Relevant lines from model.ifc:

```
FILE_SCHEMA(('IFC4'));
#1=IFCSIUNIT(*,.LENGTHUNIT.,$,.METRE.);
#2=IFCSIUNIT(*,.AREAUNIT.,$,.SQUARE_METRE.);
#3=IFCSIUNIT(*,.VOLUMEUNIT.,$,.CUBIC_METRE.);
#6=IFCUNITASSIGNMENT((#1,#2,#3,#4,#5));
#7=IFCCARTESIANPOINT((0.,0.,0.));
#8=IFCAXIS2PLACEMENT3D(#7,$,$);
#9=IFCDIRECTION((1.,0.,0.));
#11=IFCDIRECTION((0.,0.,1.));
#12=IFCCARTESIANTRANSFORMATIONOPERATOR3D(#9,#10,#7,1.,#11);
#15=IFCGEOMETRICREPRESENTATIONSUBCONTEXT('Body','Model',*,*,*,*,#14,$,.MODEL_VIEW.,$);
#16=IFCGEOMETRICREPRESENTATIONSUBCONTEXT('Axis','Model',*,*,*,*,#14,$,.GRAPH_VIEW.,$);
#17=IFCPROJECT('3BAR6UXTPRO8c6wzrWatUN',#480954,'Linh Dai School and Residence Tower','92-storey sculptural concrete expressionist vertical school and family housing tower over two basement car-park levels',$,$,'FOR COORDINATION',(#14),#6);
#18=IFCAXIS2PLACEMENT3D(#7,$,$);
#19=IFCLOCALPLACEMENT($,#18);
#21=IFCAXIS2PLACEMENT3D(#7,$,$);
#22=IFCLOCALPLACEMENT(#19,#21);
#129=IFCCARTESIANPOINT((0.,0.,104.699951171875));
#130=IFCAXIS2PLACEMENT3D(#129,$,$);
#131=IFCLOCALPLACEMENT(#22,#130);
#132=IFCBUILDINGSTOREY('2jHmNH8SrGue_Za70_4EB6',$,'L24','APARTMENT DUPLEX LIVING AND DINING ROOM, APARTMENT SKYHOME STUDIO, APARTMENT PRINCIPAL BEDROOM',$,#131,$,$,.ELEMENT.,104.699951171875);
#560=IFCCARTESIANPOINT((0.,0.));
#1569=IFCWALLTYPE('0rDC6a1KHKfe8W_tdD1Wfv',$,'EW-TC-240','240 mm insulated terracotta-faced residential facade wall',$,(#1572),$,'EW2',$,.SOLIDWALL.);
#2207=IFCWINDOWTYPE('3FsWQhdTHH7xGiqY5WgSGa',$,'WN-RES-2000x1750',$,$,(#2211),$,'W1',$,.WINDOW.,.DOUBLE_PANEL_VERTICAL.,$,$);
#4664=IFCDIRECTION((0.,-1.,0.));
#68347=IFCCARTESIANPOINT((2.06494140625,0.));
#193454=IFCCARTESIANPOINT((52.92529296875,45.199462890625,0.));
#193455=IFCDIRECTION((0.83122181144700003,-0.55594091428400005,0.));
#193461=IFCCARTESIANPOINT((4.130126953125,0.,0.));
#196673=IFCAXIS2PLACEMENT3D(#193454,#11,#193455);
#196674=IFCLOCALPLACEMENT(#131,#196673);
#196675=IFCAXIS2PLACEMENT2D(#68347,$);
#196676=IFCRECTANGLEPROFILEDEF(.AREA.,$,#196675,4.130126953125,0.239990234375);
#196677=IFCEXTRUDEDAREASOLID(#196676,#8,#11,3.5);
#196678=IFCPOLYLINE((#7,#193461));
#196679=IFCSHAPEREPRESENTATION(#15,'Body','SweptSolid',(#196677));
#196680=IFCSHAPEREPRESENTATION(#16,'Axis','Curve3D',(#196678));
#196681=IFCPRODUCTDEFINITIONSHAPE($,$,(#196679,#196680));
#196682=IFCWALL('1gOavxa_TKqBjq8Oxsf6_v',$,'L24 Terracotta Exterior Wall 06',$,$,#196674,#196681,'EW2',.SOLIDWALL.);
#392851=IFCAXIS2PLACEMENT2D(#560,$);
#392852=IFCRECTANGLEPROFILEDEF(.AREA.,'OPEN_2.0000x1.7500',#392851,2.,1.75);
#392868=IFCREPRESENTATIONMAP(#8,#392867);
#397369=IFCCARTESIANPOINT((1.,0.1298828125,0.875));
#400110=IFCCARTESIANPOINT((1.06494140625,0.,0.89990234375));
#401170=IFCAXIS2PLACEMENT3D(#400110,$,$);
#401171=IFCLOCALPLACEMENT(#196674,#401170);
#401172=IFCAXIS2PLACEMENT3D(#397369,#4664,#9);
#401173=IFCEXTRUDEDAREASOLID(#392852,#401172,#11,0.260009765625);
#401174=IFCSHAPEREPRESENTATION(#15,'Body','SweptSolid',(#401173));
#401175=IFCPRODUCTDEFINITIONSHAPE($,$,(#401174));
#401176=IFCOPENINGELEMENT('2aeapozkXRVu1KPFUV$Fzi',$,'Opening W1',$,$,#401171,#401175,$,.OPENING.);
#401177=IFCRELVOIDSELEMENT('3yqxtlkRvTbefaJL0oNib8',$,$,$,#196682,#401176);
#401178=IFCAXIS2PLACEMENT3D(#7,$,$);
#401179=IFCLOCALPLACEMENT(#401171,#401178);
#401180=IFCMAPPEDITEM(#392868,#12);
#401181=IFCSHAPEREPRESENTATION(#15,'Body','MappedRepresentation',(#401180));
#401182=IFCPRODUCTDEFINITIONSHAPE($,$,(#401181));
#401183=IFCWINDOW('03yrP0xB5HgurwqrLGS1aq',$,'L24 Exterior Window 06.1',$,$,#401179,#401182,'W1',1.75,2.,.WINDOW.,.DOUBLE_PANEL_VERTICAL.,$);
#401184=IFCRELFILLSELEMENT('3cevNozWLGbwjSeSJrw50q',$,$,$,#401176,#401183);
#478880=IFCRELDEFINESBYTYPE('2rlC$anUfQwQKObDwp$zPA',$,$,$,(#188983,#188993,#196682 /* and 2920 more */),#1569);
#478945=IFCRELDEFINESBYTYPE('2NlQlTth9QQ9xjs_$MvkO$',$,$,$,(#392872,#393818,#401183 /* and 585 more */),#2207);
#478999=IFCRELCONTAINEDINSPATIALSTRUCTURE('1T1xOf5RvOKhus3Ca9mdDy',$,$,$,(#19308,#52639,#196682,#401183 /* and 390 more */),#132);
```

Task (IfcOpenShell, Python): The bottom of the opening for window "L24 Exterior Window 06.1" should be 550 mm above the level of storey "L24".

```python
import numpy as np
import ifcopenshell
import ifcopenshell.api.geometry
import ifcopenshell.geom
import ifcopenshell.util.element
import ifcopenshell.util.placement
import ifcopenshell.util.shape
import ifcopenshell.util.unit

model = ifcopenshell.open("model.ifc")
unit_scale = ifcopenshell.util.unit.calculate_unit_scale(model)

window = model.by_guid("03yrP0xB5HgurwqrLGS1aq")
opening = window.FillsVoids[0].RelatingOpeningElement
storey = ifcopenshell.util.element.get_container(window, ifc_class="IfcBuildingStorey")
level = ifcopenshell.util.placement.get_local_placement(storey.ObjectPlacement)[2, 3]

# The opening's origin need not be at the sill, so measure its lowest point.
shape = ifcopenshell.geom.create_shape(ifcopenshell.geom.settings(), opening)
bottom = ifcopenshell.util.shape.get_shape_bottom_elevation(shape, shape.geometry) / unit_scale
dz = level + 0.55 / unit_scale - bottom

shift = np.array([0.0, 0.0, dz])
# The window is placed relative to its opening, so it follows when the opening moves.
matrix = ifcopenshell.util.placement.get_local_placement(opening.ObjectPlacement)
matrix[:3, 3] += shift
ifcopenshell.api.geometry.edit_object_placement(
    model, product=opening, matrix=matrix, is_si=False, should_transform_children=True
)

print(f"moved by {dz * unit_scale:+.3f} m")

model.write("model_v2.ifc")
```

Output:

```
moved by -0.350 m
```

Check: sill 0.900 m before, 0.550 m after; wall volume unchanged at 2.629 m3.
